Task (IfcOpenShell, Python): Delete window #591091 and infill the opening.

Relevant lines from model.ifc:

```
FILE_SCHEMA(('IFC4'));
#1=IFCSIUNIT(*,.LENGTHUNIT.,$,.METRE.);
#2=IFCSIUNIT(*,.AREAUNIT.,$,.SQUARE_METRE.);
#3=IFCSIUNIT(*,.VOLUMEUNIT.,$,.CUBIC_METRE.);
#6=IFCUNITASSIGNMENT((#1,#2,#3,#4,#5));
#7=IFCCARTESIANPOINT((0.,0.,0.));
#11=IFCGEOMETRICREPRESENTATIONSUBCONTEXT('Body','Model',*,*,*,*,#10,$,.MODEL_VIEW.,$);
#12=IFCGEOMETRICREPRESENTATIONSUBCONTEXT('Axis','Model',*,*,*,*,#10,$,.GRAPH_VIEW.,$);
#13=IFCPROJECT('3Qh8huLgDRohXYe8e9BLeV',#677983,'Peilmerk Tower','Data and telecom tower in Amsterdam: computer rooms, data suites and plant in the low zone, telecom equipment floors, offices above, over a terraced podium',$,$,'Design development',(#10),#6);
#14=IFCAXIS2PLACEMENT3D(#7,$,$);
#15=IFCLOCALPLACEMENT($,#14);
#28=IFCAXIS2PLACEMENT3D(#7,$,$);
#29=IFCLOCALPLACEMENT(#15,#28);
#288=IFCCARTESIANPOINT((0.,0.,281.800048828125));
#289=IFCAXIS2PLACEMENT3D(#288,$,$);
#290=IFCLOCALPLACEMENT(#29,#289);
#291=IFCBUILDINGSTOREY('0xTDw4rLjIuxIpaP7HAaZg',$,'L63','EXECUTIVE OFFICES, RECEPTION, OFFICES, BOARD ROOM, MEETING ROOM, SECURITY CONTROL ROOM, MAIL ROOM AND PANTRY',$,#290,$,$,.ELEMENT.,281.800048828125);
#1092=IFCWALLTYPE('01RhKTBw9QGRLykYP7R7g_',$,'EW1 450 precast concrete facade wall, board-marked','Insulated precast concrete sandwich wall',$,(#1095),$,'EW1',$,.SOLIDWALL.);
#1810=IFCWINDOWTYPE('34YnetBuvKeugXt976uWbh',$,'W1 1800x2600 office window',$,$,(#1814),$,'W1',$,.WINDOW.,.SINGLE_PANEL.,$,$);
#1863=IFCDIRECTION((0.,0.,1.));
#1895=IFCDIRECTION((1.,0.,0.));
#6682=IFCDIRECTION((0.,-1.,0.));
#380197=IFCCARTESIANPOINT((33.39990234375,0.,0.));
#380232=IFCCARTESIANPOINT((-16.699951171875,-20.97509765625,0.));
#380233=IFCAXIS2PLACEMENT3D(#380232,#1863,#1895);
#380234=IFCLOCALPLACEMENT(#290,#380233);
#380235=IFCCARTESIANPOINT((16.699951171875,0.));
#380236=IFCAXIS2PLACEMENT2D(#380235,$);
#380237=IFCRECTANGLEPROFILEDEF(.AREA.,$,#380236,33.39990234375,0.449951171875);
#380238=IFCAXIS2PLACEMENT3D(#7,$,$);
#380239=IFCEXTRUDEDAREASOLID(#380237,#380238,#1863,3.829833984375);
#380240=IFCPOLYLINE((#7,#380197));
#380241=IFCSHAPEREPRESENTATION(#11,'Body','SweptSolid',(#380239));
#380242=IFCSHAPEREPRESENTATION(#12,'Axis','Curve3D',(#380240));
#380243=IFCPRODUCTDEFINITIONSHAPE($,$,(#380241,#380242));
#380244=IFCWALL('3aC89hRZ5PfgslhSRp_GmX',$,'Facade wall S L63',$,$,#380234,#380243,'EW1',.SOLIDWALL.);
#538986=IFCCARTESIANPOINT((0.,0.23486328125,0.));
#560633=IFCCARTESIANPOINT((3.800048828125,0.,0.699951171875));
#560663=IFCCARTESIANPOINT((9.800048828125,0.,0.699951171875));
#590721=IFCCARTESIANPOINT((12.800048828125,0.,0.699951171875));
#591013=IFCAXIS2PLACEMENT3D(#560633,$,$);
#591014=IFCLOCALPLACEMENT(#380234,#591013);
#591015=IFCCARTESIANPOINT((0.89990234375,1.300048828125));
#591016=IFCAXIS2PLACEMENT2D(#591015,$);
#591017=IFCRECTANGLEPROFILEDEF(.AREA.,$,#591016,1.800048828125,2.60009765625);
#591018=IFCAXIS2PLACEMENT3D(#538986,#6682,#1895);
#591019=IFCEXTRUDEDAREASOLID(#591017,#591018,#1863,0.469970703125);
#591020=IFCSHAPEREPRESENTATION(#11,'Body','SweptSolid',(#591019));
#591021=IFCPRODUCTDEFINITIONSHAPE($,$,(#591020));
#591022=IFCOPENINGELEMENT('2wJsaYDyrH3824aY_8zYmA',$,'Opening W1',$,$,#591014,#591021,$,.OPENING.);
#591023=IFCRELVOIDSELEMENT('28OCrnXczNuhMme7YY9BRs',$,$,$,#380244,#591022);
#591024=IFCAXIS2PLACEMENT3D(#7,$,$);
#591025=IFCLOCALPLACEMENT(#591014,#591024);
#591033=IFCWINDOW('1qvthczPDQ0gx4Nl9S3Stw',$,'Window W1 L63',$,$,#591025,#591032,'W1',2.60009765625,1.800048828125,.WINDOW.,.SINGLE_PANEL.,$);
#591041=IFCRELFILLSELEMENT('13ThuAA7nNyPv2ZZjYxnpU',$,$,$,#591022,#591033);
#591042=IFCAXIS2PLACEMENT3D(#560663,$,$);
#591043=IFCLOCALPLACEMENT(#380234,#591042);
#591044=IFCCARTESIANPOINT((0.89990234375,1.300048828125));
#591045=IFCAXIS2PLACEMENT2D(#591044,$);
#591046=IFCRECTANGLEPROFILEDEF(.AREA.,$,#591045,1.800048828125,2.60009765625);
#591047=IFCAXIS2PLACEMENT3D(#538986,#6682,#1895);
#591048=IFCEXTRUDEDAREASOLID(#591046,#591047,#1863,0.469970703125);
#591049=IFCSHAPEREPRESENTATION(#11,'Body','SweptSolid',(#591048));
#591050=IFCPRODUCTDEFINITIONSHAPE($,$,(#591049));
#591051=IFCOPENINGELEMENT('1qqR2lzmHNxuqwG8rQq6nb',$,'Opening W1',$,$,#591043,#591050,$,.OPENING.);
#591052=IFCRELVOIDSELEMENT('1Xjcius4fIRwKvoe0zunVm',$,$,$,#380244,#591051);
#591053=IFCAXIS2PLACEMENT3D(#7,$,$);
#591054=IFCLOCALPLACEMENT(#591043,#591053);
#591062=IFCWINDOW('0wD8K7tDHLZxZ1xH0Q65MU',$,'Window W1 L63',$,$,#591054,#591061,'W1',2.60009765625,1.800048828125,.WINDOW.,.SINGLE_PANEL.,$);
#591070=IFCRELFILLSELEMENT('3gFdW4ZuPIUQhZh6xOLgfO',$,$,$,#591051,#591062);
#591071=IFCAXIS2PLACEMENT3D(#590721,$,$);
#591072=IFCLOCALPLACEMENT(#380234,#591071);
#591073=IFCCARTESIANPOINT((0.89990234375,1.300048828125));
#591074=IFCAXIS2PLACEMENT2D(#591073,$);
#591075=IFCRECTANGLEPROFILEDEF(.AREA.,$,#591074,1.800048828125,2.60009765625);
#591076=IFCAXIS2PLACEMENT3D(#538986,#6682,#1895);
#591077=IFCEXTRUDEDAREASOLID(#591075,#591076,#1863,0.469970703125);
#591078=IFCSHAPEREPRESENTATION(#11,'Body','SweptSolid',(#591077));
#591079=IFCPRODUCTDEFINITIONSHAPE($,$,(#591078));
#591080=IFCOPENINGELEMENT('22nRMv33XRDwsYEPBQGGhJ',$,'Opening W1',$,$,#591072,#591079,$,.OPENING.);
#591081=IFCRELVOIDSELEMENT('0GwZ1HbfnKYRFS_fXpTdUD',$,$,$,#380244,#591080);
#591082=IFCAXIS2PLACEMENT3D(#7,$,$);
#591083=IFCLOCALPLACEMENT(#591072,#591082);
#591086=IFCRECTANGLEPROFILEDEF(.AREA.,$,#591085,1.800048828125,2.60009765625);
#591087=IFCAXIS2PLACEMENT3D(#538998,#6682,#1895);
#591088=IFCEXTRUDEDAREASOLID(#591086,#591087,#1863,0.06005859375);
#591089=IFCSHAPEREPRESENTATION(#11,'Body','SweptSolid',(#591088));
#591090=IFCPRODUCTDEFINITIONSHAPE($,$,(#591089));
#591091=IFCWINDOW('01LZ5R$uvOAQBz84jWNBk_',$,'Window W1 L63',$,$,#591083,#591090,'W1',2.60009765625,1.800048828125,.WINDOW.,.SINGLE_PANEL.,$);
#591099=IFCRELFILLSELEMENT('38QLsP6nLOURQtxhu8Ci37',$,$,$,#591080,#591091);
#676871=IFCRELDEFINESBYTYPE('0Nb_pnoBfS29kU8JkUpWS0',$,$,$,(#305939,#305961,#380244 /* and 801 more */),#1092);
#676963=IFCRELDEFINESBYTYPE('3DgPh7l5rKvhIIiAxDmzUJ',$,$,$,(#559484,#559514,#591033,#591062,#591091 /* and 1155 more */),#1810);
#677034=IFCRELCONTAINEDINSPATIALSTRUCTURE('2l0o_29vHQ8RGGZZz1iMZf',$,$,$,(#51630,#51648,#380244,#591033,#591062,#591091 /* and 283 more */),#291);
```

```python
import ifcopenshell
import ifcopenshell.api.feature
import ifcopenshell.api.root
import ifcopenshell.geom
import ifcopenshell.util.shape

model = ifcopenshell.open("model.ifc")
settings = ifcopenshell.geom.settings()


def volume(element):
    """Net volume in cubic metres, openings subtracted."""
    shape = ifcopenshell.geom.create_shape(settings, element)
    return ifcopenshell.util.shape.get_volume(shape.geometry)


window = model.by_guid("01LZ5R$uvOAQBz84jWNBk_")
opening = window.FillsVoids[0].RelatingOpeningElement
wall = opening.VoidsElements[0].RelatingBuildingElement
before = volume(wall)

ifcopenshell.api.root.remove_product(model, product=window)
ifcopenshell.api.feature.remove_feature(model, feature=opening)

after = volume(wall)

print(f"wall volume {before:.3f} -> {after:.3f} m3")

model.write("model_edited.ifc")
```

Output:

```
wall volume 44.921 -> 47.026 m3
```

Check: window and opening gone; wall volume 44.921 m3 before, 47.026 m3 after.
